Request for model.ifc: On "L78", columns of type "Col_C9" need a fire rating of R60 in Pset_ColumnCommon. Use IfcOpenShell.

First a look at what the model holds.

```python
import ifcopenshell
import ifcopenshell.util.element

model = ifcopenshell.open("model.ifc")
print(model.schema)
storey = next(s for s in model.by_type("IfcBuildingStorey") if s.Name == "L78")
columns = [e for e in ifcopenshell.util.element.get_decomposition(storey) if e.is_a("IfcColumn")]
seen = {}
for e in columns:
    element_type = ifcopenshell.util.element.get_type(e)
    key = (element_type.Name if element_type != e and element_type else None, ifcopenshell.util.element.get_pset(e, "Pset_ColumnCommon", "FireRating"))
    seen[key] = seen.get(key, 0) + 1
for (name, value), count in sorted(seen.items(), key=str):
    print(count, "x", name, "|", value)
```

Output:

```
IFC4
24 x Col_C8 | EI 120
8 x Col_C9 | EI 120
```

```python
import ifcopenshell
import ifcopenshell.api.pset
import ifcopenshell.util.element

model = ifcopenshell.open("model.ifc")

storey = next(s for s in model.by_type("IfcBuildingStorey") if s.Name == "L78")
columns = [e for e in ifcopenshell.util.element.get_decomposition(storey) if e.is_a("IfcColumn")]

count = 0
for e in columns:
    element_type = ifcopenshell.util.element.get_type(e)
    if element_type in (None, e) or element_type.Name != "Col_C9":
        continue
    found = ifcopenshell.util.element.get_pset(e, "Pset_ColumnCommon", should_inherit=False)
    if found:
        pset = model.by_id(found["id"])
        if len(ifcopenshell.util.element.get_elements_by_pset(pset)) > 1:
            pset = ifcopenshell.api.pset.unshare_pset(model, products=[e], pset=pset)[0]
    else:
        pset = ifcopenshell.api.pset.add_pset(model, product=e, name="Pset_ColumnCommon")
    ifcopenshell.api.pset.edit_pset(model, pset=pset, properties={"FireRating": "R60"})
    count += 1

print(count, "columns updated")

model.write("model_edited.ifc")
```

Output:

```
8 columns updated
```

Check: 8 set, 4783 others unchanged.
